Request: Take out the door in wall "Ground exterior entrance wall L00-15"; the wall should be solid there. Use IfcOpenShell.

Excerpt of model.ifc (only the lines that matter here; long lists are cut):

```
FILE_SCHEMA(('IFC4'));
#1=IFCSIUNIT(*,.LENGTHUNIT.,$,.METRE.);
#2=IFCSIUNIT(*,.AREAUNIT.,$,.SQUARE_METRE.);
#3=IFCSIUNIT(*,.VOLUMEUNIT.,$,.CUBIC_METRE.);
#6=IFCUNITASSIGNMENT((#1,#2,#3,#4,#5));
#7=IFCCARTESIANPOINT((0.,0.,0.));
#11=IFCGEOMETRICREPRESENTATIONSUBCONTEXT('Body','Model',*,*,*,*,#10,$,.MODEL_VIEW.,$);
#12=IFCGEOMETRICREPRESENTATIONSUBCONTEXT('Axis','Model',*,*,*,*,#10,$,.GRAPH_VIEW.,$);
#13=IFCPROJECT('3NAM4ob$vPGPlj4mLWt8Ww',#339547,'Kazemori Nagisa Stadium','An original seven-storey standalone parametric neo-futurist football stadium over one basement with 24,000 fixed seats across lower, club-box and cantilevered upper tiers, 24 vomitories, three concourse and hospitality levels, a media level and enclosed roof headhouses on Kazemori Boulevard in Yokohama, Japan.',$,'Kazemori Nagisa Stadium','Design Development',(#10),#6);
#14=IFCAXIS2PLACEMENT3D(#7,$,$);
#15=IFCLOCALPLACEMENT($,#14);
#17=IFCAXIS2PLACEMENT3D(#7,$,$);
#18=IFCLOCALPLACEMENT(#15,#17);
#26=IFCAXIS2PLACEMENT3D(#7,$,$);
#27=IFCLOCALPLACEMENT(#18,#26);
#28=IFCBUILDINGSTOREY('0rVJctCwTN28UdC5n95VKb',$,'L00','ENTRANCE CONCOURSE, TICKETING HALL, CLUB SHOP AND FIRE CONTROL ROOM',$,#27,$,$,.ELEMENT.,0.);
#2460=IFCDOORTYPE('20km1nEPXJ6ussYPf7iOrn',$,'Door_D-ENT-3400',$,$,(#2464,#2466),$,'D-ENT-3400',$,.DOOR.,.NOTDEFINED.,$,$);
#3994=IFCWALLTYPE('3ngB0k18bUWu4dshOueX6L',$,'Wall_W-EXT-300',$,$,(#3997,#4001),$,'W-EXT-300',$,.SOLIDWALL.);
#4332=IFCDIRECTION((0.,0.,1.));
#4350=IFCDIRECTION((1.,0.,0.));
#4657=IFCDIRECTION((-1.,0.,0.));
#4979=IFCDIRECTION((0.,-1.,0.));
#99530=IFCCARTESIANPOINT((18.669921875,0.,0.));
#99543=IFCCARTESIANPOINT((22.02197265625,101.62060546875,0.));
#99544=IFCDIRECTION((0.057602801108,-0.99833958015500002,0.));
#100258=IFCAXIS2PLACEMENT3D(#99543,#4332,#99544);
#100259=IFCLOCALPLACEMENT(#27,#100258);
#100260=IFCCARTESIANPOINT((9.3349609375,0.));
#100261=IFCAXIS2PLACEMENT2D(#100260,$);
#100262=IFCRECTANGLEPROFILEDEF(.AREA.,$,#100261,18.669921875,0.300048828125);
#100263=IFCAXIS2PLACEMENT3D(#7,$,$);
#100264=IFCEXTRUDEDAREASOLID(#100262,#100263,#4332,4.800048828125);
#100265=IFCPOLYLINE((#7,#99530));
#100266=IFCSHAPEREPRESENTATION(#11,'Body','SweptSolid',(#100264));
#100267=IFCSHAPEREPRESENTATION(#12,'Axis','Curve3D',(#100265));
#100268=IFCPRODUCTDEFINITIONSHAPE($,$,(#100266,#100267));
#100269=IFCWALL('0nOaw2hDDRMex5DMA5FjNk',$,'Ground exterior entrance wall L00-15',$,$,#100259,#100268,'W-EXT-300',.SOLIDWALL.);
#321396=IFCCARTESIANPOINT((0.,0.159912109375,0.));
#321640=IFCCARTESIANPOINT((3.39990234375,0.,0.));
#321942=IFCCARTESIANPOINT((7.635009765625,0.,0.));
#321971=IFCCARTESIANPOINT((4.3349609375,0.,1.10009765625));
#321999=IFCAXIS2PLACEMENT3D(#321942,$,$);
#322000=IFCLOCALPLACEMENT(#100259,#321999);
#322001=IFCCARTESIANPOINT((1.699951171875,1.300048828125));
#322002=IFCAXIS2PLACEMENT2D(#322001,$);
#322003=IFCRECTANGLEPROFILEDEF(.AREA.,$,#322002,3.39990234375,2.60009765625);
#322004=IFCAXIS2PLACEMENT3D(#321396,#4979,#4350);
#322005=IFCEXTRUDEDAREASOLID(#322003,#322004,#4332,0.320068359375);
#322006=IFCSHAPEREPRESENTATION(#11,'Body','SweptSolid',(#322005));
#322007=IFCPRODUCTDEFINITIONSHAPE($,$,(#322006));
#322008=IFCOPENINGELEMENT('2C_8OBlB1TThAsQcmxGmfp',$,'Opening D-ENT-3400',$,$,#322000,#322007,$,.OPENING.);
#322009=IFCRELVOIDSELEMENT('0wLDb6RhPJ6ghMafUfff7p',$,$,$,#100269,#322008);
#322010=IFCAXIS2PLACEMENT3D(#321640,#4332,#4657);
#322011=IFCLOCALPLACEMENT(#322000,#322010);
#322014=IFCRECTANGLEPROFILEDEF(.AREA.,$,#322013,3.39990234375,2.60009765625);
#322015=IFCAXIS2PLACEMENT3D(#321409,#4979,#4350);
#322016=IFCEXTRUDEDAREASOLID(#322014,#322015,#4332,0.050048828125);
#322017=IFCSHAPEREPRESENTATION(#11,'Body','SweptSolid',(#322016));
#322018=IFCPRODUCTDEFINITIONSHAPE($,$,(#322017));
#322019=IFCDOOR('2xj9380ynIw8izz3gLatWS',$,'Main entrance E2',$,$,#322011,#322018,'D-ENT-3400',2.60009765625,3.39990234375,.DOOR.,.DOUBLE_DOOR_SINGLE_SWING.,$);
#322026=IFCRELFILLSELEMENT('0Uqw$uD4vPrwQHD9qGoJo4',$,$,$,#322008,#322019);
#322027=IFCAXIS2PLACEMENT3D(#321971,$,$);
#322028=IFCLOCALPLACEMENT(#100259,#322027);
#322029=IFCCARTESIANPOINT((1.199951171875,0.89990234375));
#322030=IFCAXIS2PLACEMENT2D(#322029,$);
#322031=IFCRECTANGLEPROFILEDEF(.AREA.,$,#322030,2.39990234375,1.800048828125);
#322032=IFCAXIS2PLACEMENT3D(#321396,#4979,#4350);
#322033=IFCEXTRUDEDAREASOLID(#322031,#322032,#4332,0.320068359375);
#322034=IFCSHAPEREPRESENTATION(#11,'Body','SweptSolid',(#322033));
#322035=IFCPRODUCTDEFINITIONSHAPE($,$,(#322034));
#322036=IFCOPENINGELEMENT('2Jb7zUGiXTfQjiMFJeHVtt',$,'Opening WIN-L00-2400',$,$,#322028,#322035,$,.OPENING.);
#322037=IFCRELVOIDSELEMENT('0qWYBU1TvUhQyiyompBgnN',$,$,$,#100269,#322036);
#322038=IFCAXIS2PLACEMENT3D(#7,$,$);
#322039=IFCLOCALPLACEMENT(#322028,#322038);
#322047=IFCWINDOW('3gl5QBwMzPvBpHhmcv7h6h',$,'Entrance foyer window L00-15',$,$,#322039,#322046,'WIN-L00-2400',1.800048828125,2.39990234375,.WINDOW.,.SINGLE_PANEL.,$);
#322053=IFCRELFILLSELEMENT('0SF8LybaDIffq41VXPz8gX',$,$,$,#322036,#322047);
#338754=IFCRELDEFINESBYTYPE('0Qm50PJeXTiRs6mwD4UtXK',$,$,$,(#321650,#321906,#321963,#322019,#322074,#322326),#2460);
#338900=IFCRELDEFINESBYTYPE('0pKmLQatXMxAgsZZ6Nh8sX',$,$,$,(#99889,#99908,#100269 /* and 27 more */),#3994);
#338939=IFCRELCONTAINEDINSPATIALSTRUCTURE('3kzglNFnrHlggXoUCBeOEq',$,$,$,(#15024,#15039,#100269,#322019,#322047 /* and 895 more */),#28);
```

```python
import ifcopenshell
import ifcopenshell.api.feature
import ifcopenshell.api.root
import ifcopenshell.geom
import ifcopenshell.util.shape

model = ifcopenshell.open("model.ifc")
settings = ifcopenshell.geom.settings()


def volume(element):
    """Net volume in cubic metres, openings subtracted."""
    shape = ifcopenshell.geom.create_shape(settings, element)
    return ifcopenshell.util.shape.get_volume(shape.geometry)


door = model.by_guid("2xj9380ynIw8izz3gLatWS")
opening = door.FillsVoids[0].RelatingOpeningElement
wall = opening.VoidsElements[0].RelatingBuildingElement
before = volume(wall)

ifcopenshell.api.root.remove_product(model, product=door)
ifcopenshell.api.feature.remove_feature(model, feature=opening)

after = volume(wall)

print(f"wall volume {before:.3f} -> {after:.3f} m3")

model.write("model_updated.ifc")
```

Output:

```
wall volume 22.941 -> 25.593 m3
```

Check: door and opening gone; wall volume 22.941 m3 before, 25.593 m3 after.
